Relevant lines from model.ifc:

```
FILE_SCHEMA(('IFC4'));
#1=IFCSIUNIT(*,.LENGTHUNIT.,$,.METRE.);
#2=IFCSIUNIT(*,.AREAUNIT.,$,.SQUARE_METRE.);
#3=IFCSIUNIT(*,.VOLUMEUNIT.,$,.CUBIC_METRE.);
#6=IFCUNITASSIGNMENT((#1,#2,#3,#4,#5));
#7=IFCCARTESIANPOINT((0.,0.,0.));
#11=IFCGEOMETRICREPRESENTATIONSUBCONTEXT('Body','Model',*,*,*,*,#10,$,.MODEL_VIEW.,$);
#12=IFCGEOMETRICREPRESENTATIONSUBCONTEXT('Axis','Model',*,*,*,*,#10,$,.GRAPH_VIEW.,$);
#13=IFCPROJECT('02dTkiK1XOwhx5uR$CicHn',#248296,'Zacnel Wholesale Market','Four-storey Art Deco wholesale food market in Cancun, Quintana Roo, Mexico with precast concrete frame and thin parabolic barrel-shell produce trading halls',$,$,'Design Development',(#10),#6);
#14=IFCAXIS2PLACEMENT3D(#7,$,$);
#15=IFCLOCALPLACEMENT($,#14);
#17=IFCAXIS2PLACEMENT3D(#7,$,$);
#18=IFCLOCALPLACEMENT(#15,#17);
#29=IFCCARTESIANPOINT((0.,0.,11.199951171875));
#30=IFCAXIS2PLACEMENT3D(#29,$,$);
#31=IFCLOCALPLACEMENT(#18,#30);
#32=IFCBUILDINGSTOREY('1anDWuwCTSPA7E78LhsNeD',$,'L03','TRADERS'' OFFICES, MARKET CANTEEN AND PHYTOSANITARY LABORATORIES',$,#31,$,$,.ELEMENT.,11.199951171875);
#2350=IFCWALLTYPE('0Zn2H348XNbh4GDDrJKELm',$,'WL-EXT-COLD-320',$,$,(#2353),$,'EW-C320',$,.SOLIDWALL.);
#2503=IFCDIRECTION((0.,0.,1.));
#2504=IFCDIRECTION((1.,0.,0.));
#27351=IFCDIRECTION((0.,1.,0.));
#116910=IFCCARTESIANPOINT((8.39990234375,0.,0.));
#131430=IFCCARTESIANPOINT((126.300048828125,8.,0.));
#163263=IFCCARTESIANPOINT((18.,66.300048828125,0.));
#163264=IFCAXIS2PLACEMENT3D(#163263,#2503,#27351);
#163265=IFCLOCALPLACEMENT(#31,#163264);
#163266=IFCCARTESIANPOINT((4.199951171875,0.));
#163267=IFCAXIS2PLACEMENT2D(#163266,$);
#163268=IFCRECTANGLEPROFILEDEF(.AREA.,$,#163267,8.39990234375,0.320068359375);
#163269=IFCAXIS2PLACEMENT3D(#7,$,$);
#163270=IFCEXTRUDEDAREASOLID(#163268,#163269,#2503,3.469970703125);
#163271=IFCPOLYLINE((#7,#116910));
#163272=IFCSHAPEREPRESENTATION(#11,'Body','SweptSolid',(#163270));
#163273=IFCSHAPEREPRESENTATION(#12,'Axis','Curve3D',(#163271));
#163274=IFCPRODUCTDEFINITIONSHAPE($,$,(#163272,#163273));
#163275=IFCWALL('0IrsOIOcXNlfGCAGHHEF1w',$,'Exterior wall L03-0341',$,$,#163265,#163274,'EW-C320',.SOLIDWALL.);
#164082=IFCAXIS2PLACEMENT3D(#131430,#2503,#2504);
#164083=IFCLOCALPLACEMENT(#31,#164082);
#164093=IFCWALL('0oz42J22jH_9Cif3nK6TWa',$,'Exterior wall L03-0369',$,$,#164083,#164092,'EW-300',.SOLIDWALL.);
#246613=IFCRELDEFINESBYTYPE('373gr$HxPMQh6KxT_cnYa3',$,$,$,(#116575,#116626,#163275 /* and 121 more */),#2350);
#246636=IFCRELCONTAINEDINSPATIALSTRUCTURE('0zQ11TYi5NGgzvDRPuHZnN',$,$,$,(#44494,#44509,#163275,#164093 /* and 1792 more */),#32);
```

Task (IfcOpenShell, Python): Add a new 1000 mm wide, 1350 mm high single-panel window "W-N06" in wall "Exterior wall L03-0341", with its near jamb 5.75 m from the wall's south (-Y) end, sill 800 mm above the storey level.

```python
import numpy as np
import ifcopenshell
import ifcopenshell.api.feature
import ifcopenshell.api.geometry
import ifcopenshell.api.root
import ifcopenshell.api.spatial
import ifcopenshell.geom
import ifcopenshell.util.element
import ifcopenshell.util.placement
import ifcopenshell.util.representation
import ifcopenshell.util.shape
import ifcopenshell.util.unit

model = ifcopenshell.open("model.ifc")
unit_scale = ifcopenshell.util.unit.calculate_unit_scale(model)
settings = ifcopenshell.geom.settings()


def volume(element):
    """Net volume in cubic metres, openings subtracted."""
    shape = ifcopenshell.geom.create_shape(settings, element)
    return ifcopenshell.util.shape.get_volume(shape.geometry)


wall = model.by_guid("0IrsOIOcXNlfGCAGHHEF1w")
storey = ifcopenshell.util.element.get_container(wall, ifc_class="IfcBuildingStorey")
context = ifcopenshell.util.representation.get_context(model, "Model", "Body", "MODEL_VIEW")
before = volume(wall)

width, height, from_end, sill = 1, 1.35, 5.75, 0.8  # metres

# The wall runs along its own X axis, and the end named is its -X end.
wall_shape = ifcopenshell.geom.create_shape(settings, wall)
x, y, z = ifcopenshell.util.shape.get_vertices(wall_shape.geometry).T
start = x.min() + from_end
face, thickness = float(y.min()), float(y.max() - y.min())
wall_matrix = ifcopenshell.util.placement.get_local_placement(wall.ObjectPlacement)
level = ifcopenshell.util.placement.get_local_placement(storey.ObjectPlacement)[2, 3]


def in_wall(x, y):
    """Placement at x, y metres in the wall's axes, at sill height."""
    matrix = wall_matrix.copy()
    matrix[:, 3] = wall_matrix @ np.array([x / unit_scale, y / unit_scale, 0.0, 1.0])
    matrix[2, 3] = level + sill / unit_scale
    return matrix


# Opening: a box that overshoots both wall faces by 50 mm.
opening = ifcopenshell.api.root.create_entity(model, ifc_class="IfcOpeningElement", predefined_type="OPENING")
box = ifcopenshell.api.geometry.add_wall_representation(
    model, context=context, length=width, height=height, thickness=thickness + 0.1
)
ifcopenshell.api.geometry.assign_representation(model, product=opening, representation=box)
ifcopenshell.api.geometry.edit_object_placement(model, product=opening, matrix=in_wall(start, face - 0.05), is_si=False)
ifcopenshell.api.feature.add_feature(model, feature=opening, element=wall)

window = ifcopenshell.api.root.create_entity(model, ifc_class="IfcWindow", name="W-N06", predefined_type="WINDOW")
window.OverallWidth, window.OverallHeight = width / unit_scale, height / unit_scale
window.PartitioningType = "SINGLE_PANEL"
body = ifcopenshell.api.geometry.add_window_representation(
    model,
    context=context,
    overall_width=window.OverallWidth,
    overall_height=window.OverallHeight,
    partition_type="SINGLE_PANEL",
)
ifcopenshell.api.geometry.assign_representation(model, product=window, representation=body)
ifcopenshell.api.spatial.assign_container(model, products=[window], relating_structure=storey)
ifcopenshell.api.feature.add_filling(model, opening=opening, element=window)

# Centre the window in the wall's thickness.
ifcopenshell.api.geometry.edit_object_placement(model, product=window, matrix=in_wall(start, face), is_si=False)
window_shape = ifcopenshell.geom.create_shape(settings, window)
depth = ifcopenshell.util.shape.get_vertices(window_shape.geometry)[:, 1]
offset = face + thickness / 2 - (depth.min() + depth.max()) / 2
ifcopenshell.api.geometry.edit_object_placement(model, product=window, matrix=in_wall(start, offset), is_si=False)

after = volume(wall)

print(f"wall volume {before:.3f} -> {after:.3f} m3")

model.write("model_updated.ifc")
```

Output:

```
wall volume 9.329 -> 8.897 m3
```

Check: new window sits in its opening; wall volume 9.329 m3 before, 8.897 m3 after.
